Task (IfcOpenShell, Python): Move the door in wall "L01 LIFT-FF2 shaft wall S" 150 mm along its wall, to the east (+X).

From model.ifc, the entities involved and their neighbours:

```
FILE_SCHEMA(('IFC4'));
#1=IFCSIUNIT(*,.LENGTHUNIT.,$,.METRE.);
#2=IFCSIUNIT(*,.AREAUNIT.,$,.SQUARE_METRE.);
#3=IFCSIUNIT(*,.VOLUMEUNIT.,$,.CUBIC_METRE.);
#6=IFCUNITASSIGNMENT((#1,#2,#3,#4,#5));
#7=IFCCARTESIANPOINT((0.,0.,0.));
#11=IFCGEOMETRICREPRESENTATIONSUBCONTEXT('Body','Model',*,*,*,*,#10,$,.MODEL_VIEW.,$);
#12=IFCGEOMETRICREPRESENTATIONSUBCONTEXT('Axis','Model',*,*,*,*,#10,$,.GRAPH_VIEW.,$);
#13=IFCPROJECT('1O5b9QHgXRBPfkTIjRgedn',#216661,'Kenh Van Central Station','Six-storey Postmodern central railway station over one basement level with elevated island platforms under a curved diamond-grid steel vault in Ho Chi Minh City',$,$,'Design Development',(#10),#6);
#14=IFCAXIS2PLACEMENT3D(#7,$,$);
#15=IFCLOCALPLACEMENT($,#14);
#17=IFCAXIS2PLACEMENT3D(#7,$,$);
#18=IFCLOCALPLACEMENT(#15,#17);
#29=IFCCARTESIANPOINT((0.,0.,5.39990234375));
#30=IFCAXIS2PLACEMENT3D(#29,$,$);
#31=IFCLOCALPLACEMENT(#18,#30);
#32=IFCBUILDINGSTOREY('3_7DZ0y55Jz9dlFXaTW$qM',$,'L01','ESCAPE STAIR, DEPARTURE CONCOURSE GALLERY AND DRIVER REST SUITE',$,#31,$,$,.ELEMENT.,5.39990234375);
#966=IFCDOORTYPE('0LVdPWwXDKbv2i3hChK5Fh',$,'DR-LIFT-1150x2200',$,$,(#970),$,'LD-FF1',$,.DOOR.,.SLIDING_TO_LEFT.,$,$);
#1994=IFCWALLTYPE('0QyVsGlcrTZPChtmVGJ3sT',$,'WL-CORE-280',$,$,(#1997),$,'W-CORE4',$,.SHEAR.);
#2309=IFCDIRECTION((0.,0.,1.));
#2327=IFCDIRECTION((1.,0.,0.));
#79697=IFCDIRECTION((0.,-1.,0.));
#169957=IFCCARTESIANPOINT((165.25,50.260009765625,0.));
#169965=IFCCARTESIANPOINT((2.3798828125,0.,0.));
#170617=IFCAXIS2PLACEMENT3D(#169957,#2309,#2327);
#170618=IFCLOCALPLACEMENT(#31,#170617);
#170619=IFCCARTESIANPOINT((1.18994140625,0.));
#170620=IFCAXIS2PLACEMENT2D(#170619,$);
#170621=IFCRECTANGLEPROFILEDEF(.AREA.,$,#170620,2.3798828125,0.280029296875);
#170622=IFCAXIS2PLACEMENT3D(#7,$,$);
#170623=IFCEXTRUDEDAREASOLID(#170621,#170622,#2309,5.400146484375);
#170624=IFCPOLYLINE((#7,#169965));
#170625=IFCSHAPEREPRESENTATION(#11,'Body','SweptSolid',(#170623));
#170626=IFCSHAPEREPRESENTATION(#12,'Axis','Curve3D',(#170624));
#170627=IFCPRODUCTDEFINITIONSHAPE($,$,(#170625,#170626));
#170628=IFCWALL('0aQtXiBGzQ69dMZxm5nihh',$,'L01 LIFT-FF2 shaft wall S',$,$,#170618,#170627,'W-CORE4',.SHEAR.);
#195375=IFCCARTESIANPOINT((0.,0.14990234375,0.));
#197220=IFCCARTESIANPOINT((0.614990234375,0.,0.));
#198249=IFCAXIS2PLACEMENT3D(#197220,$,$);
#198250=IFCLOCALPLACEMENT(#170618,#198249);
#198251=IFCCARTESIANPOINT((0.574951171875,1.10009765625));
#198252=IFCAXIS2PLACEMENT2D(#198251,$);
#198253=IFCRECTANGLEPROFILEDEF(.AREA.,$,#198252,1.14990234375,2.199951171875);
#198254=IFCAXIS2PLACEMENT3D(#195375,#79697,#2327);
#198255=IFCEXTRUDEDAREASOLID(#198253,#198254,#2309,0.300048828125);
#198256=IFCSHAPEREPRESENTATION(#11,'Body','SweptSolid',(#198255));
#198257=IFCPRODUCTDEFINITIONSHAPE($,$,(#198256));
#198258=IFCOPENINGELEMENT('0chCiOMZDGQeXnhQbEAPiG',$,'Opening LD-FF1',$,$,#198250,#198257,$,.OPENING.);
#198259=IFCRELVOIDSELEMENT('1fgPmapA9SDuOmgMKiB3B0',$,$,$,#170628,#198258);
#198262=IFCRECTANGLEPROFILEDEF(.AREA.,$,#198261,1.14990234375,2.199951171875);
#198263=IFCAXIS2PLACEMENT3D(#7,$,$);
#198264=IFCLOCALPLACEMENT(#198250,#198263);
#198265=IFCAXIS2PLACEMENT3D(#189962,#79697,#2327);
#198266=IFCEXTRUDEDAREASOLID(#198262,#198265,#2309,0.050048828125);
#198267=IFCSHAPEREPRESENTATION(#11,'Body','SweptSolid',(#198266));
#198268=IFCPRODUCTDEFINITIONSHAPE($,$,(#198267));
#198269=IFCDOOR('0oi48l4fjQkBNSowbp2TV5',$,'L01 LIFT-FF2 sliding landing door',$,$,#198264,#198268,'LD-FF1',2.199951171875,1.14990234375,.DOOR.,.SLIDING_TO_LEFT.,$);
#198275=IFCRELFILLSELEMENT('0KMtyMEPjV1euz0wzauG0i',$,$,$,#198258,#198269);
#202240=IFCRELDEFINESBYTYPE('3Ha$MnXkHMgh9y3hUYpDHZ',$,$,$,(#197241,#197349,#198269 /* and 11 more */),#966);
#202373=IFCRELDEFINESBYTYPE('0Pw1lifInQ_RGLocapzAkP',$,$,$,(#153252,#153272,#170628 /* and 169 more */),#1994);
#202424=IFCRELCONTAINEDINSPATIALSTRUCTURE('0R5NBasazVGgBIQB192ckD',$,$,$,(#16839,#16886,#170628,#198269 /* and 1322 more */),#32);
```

```python
import ifcopenshell
import ifcopenshell.api.geometry
import ifcopenshell.util.placement

model = ifcopenshell.open("model.ifc")

door = model.by_id(198269)
opening = door.FillsVoids[0].RelatingOpeningElement
wall = opening.VoidsElements[0].RelatingBuildingElement

wall_matrix = ifcopenshell.util.placement.get_local_placement(wall.ObjectPlacement)
shift = wall_matrix[:3, 0] * 0.15
before = ifcopenshell.util.placement.get_local_placement(door.ObjectPlacement)[:3, 3].copy()

# The door is placed relative to its opening, so it follows when the opening moves.
matrix = ifcopenshell.util.placement.get_local_placement(opening.ObjectPlacement)
matrix[:3, 3] += shift
ifcopenshell.api.geometry.edit_object_placement(
    model, product=opening, matrix=matrix, is_si=False, should_transform_children=True
)

after = ifcopenshell.util.placement.get_local_placement(door.ObjectPlacement)[:3, 3]
print("door moved by", (after - before).round(3) + 0.0)

model.write("model_rev.ifc")
```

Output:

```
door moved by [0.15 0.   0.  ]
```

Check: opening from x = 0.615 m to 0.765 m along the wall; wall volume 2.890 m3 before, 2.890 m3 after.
